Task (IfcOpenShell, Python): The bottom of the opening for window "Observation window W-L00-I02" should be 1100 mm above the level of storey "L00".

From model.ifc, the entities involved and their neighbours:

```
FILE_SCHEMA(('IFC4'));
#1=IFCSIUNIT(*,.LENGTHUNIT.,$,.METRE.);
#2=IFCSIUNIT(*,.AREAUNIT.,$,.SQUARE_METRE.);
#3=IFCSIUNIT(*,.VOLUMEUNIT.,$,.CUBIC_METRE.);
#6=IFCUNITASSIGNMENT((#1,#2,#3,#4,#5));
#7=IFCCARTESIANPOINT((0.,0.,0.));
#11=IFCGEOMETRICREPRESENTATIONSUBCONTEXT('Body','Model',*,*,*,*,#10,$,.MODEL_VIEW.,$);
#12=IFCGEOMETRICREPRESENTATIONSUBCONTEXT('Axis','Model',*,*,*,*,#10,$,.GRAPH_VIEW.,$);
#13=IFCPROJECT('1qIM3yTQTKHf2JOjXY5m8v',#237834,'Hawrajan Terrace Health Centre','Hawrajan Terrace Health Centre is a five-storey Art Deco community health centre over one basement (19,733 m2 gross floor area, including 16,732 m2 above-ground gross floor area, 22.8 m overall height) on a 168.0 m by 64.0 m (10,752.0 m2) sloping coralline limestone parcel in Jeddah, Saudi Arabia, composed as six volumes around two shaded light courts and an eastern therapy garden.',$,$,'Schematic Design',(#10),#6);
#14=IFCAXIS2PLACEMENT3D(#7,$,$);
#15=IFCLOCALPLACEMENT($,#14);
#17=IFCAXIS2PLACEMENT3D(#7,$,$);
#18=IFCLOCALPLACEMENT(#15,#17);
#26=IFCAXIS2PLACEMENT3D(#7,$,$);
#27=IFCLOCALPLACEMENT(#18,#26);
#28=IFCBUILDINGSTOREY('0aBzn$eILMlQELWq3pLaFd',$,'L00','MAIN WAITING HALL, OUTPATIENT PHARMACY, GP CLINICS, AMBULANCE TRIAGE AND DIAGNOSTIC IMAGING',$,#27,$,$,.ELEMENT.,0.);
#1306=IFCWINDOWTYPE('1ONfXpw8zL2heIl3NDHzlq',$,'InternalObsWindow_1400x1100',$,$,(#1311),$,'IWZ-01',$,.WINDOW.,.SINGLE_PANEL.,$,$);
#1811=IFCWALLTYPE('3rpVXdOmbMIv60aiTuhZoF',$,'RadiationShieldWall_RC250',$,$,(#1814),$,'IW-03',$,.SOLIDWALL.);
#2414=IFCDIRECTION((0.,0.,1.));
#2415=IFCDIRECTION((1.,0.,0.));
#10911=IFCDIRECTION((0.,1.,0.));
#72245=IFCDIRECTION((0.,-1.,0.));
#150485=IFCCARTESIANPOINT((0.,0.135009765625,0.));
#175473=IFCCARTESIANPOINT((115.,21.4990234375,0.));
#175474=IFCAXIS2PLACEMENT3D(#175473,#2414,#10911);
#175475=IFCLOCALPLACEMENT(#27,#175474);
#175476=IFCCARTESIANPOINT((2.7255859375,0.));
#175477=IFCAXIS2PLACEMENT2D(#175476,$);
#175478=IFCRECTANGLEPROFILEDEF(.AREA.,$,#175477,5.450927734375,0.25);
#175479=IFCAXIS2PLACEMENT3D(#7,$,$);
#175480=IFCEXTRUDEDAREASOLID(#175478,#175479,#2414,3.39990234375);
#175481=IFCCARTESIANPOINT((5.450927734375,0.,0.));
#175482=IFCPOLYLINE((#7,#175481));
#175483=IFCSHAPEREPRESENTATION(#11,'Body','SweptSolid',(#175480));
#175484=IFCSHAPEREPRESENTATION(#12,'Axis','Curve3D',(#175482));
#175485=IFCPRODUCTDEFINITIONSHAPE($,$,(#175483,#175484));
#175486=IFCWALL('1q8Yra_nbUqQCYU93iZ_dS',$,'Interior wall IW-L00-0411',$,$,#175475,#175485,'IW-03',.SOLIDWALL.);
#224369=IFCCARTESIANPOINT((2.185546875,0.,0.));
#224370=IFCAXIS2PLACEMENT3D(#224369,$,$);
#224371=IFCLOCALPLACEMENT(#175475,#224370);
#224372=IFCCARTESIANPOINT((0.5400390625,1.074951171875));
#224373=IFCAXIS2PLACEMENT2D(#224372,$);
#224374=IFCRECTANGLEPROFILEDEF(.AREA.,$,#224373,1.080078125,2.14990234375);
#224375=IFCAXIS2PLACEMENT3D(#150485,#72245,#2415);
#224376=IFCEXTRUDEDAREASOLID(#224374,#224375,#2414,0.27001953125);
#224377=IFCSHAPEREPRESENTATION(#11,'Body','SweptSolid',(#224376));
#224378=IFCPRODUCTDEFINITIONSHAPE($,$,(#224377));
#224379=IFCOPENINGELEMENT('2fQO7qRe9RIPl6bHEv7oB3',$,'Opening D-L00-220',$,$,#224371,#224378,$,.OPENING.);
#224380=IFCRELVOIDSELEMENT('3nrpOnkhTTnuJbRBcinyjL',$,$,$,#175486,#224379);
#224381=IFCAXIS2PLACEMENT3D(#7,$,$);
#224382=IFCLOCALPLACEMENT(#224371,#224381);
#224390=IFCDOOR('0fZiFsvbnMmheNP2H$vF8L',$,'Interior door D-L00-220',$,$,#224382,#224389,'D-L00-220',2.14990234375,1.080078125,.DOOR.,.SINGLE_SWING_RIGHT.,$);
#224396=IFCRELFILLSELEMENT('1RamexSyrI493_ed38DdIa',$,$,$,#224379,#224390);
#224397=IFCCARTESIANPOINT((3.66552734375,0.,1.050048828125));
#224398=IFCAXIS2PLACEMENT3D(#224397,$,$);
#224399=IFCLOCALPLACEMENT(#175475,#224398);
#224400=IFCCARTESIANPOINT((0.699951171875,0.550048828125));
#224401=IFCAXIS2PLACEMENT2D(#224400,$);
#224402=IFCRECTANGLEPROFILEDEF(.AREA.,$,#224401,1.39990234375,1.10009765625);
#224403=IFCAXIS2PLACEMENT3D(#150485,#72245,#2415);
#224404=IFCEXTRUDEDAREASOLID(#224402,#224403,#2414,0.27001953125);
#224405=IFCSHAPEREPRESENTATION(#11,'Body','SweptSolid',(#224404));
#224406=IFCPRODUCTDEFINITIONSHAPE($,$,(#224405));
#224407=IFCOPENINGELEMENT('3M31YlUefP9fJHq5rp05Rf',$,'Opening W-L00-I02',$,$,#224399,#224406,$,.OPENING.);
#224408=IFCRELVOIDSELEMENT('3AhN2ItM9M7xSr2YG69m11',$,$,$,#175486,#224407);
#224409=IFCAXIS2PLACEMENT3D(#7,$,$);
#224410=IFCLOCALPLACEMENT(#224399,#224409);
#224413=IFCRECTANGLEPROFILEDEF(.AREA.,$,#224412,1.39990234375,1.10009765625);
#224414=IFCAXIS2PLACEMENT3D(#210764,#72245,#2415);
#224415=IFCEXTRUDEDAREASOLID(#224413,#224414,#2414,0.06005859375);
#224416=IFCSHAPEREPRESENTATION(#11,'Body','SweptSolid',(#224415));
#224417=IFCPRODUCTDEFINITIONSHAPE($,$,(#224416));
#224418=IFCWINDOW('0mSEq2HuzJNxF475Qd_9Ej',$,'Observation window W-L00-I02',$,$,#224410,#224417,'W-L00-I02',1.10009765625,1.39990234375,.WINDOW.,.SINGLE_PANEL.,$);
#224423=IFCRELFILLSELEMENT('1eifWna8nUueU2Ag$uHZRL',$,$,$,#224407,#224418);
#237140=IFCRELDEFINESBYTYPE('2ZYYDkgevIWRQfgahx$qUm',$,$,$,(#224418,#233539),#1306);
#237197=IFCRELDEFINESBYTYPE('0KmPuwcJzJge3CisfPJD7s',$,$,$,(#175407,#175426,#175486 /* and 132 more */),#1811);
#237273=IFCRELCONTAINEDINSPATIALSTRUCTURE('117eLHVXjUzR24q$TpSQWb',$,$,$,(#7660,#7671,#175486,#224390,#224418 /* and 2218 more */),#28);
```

```python
import numpy as np
import ifcopenshell
import ifcopenshell.api.geometry
import ifcopenshell.geom
import ifcopenshell.util.element
import ifcopenshell.util.placement
import ifcopenshell.util.shape
import ifcopenshell.util.unit

model = ifcopenshell.open("model.ifc")
unit_scale = ifcopenshell.util.unit.calculate_unit_scale(model)

window = model.by_id(224418)
opening = window.FillsVoids[0].RelatingOpeningElement
storey = ifcopenshell.util.element.get_container(window, ifc_class="IfcBuildingStorey")
level = ifcopenshell.util.placement.get_local_placement(storey.ObjectPlacement)[2, 3]

# The opening's origin need not be at the sill, so measure its lowest point.
shape = ifcopenshell.geom.create_shape(ifcopenshell.geom.settings(), opening)
bottom = ifcopenshell.util.shape.get_shape_bottom_elevation(shape, shape.geometry) / unit_scale
dz = level + 1.1 / unit_scale - bottom

shift = np.array([0.0, 0.0, dz])
# The window is placed relative to its opening, so it follows when the opening moves.
matrix = ifcopenshell.util.placement.get_local_placement(opening.ObjectPlacement)
matrix[:3, 3] += shift
ifcopenshell.api.geometry.edit_object_placement(
    model, product=opening, matrix=matrix, is_si=False, should_transform_children=True
)

print(f"moved by {dz * unit_scale:+.3f} m")

model.write("model_updated.ifc")
```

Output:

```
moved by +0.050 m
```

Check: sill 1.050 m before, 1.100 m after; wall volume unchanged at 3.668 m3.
